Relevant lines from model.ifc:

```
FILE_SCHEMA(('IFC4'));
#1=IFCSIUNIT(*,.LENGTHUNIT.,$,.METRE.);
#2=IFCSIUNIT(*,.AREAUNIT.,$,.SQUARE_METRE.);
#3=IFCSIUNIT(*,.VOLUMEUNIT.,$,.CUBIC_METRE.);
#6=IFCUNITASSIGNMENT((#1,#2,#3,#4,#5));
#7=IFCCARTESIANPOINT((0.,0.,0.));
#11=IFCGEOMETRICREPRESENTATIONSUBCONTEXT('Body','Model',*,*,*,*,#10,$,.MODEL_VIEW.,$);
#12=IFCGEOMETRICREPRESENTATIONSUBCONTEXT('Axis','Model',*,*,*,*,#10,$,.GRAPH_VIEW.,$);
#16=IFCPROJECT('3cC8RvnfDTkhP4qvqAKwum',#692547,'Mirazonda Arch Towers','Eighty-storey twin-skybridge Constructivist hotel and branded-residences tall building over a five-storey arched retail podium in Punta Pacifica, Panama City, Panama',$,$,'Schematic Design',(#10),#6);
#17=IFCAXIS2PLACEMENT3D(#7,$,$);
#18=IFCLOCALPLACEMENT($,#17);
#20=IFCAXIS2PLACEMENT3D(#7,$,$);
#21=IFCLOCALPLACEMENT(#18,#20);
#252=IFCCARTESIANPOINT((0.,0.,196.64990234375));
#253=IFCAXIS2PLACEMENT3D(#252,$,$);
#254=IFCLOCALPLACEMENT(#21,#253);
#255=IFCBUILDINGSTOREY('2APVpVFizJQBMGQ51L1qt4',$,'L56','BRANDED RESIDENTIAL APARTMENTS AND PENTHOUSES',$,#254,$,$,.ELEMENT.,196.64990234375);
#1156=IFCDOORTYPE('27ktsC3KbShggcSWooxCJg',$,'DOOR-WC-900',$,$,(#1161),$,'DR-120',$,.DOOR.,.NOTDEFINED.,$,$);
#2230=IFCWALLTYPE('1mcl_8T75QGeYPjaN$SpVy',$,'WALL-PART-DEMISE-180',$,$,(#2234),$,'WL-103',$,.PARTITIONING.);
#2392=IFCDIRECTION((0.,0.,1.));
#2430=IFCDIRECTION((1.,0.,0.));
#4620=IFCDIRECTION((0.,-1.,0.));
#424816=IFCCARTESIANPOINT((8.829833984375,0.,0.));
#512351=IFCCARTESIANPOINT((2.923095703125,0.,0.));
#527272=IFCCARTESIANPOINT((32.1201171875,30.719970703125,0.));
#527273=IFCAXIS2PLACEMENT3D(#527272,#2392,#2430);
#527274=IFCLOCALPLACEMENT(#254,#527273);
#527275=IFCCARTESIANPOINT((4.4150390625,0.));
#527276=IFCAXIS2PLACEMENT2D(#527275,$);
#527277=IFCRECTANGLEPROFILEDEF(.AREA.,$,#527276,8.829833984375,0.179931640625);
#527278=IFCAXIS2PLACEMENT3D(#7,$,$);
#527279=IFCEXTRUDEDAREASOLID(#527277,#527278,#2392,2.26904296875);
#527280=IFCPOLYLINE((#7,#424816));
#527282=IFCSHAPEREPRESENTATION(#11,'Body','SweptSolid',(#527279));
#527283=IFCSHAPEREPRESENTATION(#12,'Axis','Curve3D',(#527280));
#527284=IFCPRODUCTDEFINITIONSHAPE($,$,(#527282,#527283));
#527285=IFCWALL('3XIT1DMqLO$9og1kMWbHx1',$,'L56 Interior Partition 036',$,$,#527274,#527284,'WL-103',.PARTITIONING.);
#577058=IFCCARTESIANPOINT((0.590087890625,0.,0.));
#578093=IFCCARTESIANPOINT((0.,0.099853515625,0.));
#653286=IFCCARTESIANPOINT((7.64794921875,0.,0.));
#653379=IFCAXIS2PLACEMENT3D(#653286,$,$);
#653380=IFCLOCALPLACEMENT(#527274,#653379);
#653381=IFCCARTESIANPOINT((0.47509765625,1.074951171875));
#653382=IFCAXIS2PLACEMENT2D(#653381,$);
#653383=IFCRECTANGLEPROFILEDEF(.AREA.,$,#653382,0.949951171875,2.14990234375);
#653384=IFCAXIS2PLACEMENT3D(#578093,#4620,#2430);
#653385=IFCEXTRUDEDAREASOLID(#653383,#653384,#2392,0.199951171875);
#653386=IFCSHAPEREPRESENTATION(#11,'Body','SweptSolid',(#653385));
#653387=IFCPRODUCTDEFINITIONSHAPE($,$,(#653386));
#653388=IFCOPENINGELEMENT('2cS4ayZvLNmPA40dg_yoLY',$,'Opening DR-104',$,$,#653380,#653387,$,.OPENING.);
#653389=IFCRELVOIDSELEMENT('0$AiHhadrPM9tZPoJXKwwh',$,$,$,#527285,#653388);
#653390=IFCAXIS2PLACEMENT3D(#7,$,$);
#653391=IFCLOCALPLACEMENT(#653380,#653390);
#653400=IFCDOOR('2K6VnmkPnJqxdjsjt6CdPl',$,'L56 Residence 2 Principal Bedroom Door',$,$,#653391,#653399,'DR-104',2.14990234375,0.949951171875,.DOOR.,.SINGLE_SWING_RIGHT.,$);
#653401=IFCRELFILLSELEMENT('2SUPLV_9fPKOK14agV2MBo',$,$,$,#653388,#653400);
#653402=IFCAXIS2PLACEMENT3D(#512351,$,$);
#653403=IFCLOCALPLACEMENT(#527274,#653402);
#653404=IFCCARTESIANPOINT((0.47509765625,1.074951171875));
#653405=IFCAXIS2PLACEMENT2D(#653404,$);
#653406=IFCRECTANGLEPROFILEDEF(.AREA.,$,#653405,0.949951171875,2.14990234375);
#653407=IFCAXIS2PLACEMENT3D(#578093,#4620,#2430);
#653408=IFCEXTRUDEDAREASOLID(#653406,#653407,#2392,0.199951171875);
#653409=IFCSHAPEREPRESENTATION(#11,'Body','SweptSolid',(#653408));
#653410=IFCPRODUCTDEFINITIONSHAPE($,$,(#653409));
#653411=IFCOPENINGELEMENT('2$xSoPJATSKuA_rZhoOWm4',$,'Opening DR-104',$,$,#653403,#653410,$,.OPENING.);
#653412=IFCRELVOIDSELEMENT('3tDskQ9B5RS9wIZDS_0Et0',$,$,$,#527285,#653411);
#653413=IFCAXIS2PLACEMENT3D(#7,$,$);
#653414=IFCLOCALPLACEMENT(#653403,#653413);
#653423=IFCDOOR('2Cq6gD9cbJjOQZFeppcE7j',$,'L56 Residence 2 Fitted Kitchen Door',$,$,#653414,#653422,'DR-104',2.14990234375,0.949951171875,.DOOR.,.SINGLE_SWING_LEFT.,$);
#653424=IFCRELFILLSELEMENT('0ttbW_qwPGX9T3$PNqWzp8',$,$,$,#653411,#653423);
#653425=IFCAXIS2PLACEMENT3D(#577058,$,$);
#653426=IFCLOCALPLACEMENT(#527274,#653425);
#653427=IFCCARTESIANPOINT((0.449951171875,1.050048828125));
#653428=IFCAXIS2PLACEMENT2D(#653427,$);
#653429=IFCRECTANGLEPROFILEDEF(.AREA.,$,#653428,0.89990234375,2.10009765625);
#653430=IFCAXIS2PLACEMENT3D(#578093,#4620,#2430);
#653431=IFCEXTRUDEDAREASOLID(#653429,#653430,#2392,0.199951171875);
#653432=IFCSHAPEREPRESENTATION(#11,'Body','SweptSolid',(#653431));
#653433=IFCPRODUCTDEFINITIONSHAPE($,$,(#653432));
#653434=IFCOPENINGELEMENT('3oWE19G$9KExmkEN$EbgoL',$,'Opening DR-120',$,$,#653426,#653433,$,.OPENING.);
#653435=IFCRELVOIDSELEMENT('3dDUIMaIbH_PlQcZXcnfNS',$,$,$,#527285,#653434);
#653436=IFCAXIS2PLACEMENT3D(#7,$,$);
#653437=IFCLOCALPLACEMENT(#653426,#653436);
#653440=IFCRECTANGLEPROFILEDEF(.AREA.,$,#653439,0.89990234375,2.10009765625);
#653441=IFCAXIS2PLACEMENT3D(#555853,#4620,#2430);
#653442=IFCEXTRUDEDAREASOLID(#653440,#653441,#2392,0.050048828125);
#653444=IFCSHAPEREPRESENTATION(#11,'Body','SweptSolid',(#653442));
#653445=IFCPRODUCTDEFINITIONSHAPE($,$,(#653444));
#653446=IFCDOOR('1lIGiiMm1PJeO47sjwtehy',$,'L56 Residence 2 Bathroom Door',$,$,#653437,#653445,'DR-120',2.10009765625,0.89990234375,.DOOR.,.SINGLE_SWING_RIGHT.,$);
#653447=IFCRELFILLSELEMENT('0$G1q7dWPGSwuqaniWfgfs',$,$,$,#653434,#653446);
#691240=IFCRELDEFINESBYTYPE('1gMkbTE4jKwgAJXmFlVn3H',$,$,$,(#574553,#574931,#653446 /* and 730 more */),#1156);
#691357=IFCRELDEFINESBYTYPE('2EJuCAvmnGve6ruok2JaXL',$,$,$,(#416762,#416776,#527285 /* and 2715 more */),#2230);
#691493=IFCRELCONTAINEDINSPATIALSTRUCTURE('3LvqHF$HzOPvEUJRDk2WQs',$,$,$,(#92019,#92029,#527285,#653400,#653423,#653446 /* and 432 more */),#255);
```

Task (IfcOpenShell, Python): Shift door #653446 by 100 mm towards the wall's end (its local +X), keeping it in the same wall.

```python
import ifcopenshell
import ifcopenshell.api.geometry
import ifcopenshell.util.placement
import ifcopenshell.util.unit

model = ifcopenshell.open("model.ifc")
unit_scale = ifcopenshell.util.unit.calculate_unit_scale(model)

door = model.by_guid("1lIGiiMm1PJeO47sjwtehy")
opening = door.FillsVoids[0].RelatingOpeningElement
wall = opening.VoidsElements[0].RelatingBuildingElement

wall_matrix = ifcopenshell.util.placement.get_local_placement(wall.ObjectPlacement)
shift = wall_matrix[:3, 0] * 0.1 / unit_scale
before = ifcopenshell.util.placement.get_local_placement(door.ObjectPlacement)[:3, 3].copy()

# The door is placed relative to its opening, so it follows when the opening moves.
matrix = ifcopenshell.util.placement.get_local_placement(opening.ObjectPlacement)
matrix[:3, 3] += shift
ifcopenshell.api.geometry.edit_object_placement(
    model, product=opening, matrix=matrix, is_si=False, should_transform_children=True
)

after = ifcopenshell.util.placement.get_local_placement(door.ObjectPlacement)[:3, 3]
print("door moved by", (after - before).round(3) + 0.0)

model.write("model_edited.ifc")
```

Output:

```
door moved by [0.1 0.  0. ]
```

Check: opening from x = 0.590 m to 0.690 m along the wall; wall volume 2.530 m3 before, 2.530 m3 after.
